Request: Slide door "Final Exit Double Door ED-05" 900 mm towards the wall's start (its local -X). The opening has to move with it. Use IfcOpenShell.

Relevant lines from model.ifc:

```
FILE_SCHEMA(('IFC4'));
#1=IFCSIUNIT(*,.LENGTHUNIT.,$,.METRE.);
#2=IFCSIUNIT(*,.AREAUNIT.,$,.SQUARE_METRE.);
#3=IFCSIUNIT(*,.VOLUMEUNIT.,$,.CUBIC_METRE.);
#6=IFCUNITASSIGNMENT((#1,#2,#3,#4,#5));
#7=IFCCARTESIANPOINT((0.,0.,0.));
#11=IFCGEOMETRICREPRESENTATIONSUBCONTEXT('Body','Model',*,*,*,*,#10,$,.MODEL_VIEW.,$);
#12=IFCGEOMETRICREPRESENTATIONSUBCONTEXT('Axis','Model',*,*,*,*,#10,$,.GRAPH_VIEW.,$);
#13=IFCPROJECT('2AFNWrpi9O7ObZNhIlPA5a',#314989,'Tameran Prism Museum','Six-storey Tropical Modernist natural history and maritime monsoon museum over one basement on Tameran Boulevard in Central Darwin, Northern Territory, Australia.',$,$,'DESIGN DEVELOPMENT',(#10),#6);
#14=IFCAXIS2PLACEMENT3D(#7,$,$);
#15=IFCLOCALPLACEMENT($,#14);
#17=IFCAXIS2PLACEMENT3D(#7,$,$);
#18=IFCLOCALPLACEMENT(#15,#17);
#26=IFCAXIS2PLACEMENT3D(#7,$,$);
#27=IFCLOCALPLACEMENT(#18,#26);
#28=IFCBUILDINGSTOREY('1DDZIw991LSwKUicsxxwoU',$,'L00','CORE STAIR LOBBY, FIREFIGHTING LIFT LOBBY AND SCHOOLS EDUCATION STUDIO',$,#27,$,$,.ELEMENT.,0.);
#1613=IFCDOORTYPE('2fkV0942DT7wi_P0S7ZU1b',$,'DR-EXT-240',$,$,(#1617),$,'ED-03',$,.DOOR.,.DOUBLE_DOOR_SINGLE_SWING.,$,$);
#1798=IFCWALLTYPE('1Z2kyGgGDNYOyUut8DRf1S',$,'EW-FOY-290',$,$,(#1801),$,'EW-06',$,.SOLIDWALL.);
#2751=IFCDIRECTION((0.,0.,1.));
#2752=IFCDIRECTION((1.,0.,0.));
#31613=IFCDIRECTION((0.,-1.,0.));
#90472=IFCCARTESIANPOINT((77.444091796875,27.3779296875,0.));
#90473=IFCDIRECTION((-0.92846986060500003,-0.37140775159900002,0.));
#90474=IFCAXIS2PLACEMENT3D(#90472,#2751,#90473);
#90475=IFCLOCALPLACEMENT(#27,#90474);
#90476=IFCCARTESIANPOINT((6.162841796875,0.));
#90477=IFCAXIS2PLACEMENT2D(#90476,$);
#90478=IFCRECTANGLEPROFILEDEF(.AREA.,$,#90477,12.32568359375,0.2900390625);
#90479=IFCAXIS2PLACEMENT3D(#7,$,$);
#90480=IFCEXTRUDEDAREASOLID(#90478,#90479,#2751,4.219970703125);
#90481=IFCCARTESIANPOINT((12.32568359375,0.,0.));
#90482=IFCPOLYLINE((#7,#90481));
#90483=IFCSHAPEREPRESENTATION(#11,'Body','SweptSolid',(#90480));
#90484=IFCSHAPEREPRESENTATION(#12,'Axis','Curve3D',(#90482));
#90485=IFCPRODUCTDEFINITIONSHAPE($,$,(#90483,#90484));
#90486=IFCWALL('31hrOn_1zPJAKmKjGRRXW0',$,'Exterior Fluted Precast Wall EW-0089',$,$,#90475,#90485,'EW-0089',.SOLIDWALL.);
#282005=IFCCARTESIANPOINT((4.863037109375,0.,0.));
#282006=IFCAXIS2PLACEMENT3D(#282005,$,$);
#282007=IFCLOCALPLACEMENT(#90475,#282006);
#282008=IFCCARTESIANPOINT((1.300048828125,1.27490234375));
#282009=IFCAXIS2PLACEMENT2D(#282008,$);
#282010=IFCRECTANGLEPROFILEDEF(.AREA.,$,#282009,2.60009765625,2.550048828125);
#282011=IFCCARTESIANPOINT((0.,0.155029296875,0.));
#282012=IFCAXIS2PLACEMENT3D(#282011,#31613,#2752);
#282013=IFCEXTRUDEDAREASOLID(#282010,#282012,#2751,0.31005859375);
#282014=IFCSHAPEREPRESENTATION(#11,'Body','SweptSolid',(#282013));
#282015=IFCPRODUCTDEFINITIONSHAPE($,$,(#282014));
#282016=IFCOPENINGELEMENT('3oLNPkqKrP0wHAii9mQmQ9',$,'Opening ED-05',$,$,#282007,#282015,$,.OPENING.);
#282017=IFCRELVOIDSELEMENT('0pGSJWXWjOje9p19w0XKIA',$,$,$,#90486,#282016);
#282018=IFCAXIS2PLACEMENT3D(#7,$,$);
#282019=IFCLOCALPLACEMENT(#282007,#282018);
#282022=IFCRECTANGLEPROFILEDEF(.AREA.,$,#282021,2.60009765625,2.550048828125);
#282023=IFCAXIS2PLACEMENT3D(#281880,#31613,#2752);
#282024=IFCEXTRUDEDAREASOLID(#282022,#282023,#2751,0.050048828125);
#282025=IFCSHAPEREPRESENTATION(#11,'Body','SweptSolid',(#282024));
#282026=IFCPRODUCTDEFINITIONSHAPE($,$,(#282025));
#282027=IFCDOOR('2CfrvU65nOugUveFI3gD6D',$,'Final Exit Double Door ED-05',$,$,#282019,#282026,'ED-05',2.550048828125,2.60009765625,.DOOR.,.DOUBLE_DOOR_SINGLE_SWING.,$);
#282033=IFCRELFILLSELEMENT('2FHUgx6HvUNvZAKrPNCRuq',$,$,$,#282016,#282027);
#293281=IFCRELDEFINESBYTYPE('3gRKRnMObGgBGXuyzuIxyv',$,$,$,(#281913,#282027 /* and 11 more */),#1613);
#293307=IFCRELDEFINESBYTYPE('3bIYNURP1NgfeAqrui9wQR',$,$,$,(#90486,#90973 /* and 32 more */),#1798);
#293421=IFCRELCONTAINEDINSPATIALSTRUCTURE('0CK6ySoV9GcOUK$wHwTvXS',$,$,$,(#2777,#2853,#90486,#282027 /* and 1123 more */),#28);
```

```python
import ifcopenshell
import ifcopenshell.api.geometry
import ifcopenshell.util.placement
import ifcopenshell.util.unit

model = ifcopenshell.open("model.ifc")
unit_scale = ifcopenshell.util.unit.calculate_unit_scale(model)

door = model.by_guid("2CfrvU65nOugUveFI3gD6D")
opening = door.FillsVoids[0].RelatingOpeningElement
wall = opening.VoidsElements[0].RelatingBuildingElement

wall_matrix = ifcopenshell.util.placement.get_local_placement(wall.ObjectPlacement)
shift = wall_matrix[:3, 0] * -0.9 / unit_scale
before = ifcopenshell.util.placement.get_local_placement(door.ObjectPlacement)[:3, 3].copy()

# The door is placed relative to its opening, so it follows when the opening moves.
matrix = ifcopenshell.util.placement.get_local_placement(opening.ObjectPlacement)
matrix[:3, 3] += shift
ifcopenshell.api.geometry.edit_object_placement(
    model, product=opening, matrix=matrix, is_si=False, should_transform_children=True
)

after = ifcopenshell.util.placement.get_local_placement(door.ObjectPlacement)[:3, 3]
print("door moved by", (after - before).round(3) + 0.0)

model.write("model-out.ifc")
```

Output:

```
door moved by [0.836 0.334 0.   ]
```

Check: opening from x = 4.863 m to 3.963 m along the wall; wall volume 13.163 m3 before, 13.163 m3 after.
